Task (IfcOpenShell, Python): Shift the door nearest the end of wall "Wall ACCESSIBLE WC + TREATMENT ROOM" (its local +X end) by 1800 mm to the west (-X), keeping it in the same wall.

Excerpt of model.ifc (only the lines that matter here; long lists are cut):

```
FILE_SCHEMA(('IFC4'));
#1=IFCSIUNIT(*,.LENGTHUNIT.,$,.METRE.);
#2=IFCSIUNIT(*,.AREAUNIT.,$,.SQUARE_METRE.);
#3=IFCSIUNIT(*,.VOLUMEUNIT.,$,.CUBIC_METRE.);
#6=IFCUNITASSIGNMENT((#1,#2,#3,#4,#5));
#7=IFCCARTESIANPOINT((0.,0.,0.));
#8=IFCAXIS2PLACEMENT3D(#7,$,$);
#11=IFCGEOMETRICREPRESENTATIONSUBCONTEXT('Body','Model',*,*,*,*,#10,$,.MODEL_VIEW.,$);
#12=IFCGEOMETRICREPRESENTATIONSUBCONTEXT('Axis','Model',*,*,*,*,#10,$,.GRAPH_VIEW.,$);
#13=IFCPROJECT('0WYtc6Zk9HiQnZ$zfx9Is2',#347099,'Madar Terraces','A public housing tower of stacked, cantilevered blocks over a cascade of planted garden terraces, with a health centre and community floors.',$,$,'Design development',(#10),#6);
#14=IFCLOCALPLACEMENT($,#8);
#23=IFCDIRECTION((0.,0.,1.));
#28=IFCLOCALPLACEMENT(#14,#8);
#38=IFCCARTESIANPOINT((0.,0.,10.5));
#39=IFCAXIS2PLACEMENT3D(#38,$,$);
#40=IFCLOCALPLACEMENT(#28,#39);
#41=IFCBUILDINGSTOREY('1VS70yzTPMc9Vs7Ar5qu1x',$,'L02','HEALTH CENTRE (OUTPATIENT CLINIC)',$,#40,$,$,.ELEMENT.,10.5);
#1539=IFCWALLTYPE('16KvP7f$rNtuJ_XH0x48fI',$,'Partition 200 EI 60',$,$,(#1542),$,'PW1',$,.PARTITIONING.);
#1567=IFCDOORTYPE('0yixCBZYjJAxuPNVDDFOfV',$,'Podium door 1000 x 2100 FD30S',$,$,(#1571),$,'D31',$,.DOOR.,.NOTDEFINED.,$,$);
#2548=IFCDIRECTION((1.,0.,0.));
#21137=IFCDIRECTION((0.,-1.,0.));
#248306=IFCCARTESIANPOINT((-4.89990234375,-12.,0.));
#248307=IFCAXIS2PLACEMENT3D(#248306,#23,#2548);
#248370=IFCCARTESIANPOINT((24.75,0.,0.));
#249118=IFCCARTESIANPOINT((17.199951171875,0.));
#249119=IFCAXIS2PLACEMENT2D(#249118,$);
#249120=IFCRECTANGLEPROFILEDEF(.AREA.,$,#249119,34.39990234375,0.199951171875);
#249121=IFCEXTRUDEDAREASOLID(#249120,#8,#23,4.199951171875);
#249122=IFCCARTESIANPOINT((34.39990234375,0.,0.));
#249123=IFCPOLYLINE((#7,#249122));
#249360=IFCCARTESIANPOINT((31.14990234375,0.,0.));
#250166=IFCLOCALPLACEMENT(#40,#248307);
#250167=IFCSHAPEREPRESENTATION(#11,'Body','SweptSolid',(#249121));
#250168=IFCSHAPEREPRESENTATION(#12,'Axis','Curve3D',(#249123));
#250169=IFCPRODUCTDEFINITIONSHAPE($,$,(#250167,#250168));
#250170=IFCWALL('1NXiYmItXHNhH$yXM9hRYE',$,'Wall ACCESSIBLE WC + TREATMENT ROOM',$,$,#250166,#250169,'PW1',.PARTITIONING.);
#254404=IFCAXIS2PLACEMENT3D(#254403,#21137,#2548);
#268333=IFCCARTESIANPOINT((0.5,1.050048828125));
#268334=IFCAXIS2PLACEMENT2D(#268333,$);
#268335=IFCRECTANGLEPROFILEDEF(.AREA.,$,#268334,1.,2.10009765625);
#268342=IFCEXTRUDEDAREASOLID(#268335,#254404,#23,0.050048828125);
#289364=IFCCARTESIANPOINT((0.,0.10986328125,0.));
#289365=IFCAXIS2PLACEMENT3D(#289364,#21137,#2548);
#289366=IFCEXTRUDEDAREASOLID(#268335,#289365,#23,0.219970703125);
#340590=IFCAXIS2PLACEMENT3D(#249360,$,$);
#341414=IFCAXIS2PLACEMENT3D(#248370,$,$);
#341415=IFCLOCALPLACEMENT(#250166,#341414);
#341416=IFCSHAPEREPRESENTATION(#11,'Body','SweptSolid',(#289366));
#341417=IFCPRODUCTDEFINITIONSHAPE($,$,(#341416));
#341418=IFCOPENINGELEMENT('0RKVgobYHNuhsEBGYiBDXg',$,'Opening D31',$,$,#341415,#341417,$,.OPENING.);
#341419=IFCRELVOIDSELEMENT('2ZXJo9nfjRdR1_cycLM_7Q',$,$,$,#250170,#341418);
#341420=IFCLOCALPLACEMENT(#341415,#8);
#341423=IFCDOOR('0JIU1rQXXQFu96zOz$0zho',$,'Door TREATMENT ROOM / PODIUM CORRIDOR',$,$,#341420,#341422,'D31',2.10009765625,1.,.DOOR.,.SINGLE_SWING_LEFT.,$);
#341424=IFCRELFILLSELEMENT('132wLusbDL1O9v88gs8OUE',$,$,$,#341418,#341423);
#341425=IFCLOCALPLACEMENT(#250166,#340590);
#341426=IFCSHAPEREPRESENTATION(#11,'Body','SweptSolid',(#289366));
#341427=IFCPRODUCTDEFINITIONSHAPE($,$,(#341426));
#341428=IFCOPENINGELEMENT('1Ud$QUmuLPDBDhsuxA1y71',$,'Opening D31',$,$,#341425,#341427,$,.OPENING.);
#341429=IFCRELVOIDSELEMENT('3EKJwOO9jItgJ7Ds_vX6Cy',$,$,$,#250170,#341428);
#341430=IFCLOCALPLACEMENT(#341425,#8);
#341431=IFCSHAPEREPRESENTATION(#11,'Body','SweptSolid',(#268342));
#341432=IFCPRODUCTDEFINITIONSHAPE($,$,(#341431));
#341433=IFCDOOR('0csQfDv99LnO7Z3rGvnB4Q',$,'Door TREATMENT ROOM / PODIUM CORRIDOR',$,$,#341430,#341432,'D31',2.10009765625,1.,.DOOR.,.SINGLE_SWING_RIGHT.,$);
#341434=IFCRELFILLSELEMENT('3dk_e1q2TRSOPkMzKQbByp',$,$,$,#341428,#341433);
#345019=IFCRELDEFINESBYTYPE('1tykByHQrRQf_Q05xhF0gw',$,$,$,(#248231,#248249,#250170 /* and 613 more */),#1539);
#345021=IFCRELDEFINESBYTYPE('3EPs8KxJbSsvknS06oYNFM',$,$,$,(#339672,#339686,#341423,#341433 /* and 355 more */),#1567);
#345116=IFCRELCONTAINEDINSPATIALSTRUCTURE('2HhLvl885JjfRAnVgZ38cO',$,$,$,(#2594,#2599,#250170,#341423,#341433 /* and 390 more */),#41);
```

```python
import ifcopenshell
import ifcopenshell.api.geometry
import ifcopenshell.util.placement

model = ifcopenshell.open("model.ifc")

door = model.by_id(341433)
opening = door.FillsVoids[0].RelatingOpeningElement
wall = opening.VoidsElements[0].RelatingBuildingElement

wall_matrix = ifcopenshell.util.placement.get_local_placement(wall.ObjectPlacement)
shift = wall_matrix[:3, 0] * -1.8
before = ifcopenshell.util.placement.get_local_placement(door.ObjectPlacement)[:3, 3].copy()

# The door is placed relative to its opening, so it follows when the opening moves.
matrix = ifcopenshell.util.placement.get_local_placement(opening.ObjectPlacement)
matrix[:3, 3] += shift
ifcopenshell.api.geometry.edit_object_placement(
    model, product=opening, matrix=matrix, is_si=False, should_transform_children=True
)

after = ifcopenshell.util.placement.get_local_placement(door.ObjectPlacement)[:3, 3]
print("door moved by", (after - before).round(3) + 0.0)

model.write("model_rev.ifc")
```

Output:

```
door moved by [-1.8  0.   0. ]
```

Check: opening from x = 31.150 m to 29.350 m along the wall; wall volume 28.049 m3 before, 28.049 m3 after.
